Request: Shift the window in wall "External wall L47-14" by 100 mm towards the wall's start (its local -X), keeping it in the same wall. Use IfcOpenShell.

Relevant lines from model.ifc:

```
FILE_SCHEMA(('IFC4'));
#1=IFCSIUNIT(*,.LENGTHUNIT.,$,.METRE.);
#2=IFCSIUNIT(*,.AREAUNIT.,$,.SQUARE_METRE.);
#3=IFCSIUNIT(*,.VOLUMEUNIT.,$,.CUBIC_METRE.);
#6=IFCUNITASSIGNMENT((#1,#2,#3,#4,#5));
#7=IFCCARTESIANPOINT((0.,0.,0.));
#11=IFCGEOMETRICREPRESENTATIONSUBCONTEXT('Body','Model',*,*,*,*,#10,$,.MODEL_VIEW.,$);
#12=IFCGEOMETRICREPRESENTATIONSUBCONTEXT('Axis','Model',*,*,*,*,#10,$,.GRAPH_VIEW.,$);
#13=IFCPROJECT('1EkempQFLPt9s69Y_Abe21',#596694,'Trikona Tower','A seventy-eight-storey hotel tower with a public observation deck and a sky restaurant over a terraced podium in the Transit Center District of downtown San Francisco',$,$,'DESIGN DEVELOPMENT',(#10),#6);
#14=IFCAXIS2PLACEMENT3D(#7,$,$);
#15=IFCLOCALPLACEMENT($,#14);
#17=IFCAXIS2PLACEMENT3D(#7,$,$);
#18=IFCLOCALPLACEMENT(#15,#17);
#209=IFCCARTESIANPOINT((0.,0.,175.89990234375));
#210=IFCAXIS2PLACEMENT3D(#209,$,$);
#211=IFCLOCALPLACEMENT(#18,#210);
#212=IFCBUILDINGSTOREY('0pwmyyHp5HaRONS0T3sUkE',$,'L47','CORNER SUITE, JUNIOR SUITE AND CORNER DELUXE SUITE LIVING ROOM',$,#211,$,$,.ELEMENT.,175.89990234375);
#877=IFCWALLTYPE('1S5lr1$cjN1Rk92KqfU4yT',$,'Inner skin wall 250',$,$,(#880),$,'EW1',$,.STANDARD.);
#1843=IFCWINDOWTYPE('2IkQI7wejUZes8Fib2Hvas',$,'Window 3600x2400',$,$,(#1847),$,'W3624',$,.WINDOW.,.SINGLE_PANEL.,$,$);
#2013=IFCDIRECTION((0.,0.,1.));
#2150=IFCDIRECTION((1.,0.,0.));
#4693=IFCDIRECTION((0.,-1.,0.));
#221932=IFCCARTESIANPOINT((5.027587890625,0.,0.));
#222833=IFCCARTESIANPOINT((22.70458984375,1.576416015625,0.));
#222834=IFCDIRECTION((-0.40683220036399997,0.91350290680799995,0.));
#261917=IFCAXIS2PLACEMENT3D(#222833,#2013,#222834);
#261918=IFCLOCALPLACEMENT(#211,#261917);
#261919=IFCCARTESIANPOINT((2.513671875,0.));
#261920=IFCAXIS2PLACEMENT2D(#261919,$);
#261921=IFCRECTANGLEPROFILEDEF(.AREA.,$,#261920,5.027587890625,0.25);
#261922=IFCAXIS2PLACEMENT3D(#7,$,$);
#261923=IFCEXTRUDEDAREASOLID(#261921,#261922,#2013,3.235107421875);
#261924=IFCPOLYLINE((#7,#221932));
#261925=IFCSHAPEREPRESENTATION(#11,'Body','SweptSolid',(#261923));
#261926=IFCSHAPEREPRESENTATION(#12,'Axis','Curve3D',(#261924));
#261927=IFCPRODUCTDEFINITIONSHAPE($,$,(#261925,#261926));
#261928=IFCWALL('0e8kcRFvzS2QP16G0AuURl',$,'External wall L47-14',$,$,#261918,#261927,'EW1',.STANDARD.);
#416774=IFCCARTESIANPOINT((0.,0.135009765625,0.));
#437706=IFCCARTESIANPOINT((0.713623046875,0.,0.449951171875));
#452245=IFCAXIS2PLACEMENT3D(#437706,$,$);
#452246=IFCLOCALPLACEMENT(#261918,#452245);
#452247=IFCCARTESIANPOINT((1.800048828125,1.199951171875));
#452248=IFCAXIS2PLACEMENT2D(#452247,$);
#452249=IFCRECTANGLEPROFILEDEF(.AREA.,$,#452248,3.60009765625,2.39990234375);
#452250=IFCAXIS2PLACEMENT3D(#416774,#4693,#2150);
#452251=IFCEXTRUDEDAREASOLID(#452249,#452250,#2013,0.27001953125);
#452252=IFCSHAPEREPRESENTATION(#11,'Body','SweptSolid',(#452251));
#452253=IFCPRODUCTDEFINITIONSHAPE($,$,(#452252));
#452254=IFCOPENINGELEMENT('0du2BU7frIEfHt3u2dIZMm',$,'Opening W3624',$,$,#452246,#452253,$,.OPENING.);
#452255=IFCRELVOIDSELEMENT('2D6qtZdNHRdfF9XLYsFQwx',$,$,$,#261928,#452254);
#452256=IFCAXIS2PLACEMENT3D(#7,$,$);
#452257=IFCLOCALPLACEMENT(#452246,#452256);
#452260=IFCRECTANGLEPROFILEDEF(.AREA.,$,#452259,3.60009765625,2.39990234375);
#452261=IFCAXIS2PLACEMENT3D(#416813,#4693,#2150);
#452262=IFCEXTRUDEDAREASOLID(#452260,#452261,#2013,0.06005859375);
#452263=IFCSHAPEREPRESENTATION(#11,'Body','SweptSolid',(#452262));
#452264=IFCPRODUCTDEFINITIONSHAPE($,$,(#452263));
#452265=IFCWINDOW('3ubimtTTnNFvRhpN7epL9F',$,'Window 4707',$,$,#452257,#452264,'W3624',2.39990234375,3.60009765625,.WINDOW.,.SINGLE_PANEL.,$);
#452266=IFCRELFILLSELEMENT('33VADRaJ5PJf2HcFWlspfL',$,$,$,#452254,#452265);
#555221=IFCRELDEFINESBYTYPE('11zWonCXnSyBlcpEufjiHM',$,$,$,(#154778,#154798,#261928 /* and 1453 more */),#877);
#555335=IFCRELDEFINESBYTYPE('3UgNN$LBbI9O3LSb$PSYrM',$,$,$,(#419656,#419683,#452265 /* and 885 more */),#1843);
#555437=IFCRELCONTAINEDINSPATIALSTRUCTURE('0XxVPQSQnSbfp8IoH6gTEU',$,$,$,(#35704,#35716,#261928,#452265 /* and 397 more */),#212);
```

```python
import ifcopenshell
import ifcopenshell.api.geometry
import ifcopenshell.util.placement
import ifcopenshell.util.unit

model = ifcopenshell.open("model.ifc")
unit_scale = ifcopenshell.util.unit.calculate_unit_scale(model)

window = model.by_guid("3ubimtTTnNFvRhpN7epL9F")
opening = window.FillsVoids[0].RelatingOpeningElement
wall = opening.VoidsElements[0].RelatingBuildingElement

wall_matrix = ifcopenshell.util.placement.get_local_placement(wall.ObjectPlacement)
shift = wall_matrix[:3, 0] * -0.1 / unit_scale
before = ifcopenshell.util.placement.get_local_placement(window.ObjectPlacement)[:3, 3].copy()

# The window is placed relative to its opening, so it follows when the opening moves.
matrix = ifcopenshell.util.placement.get_local_placement(opening.ObjectPlacement)
matrix[:3, 3] += shift
ifcopenshell.api.geometry.edit_object_placement(
    model, product=opening, matrix=matrix, is_si=False, should_transform_children=True
)

after = ifcopenshell.util.placement.get_local_placement(window.ObjectPlacement)[:3, 3]
print("window moved by", (after - before).round(3) + 0.0)

model.write("model_edited.ifc")
```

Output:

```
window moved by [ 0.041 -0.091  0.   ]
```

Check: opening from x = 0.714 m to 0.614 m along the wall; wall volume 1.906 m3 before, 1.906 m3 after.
